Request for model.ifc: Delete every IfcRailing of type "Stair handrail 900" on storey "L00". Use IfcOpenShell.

First a look at what the model holds.

```python
import ifcopenshell
import ifcopenshell.util.element

model = ifcopenshell.open("model.ifc")
print(model.schema)
storey = next(s for s in model.by_type("IfcBuildingStorey") if s.Name == "L00")
railings = [e for e in ifcopenshell.util.element.get_decomposition(storey) if e.is_a("IfcRailing")]
seen = {}
for e in railings:
    element_type = ifcopenshell.util.element.get_type(e)
    name = element_type.Name if element_type not in (None, e) else None
    seen[name] = seen.get(name, 0) + 1
for name, count in sorted(seen.items(), key=str):
    print(count, "x", name)
```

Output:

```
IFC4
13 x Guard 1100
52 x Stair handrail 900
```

```python
import ifcopenshell
import ifcopenshell.api.root
import ifcopenshell.util.element

model = ifcopenshell.open("model.ifc")

storey = next(s for s in model.by_type("IfcBuildingStorey") if s.Name == "L00")
railings = [e for e in ifcopenshell.util.element.get_decomposition(storey) if e.is_a("IfcRailing")]
targets = [e for e in railings if (t := ifcopenshell.util.element.get_type(e)) not in (None, e) and t.Name == "Stair handrail 900"]

for e in targets:
    ifcopenshell.api.root.remove_product(model, product=e)
print(len(targets), "removed")

model.write("model_edited.ifc")
```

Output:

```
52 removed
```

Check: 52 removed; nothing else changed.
